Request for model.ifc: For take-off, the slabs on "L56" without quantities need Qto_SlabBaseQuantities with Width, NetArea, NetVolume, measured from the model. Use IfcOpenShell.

First a look at what the model holds.

```python
import ifcopenshell
import ifcopenshell.util.element
import ifcopenshell.util.unit

model = ifcopenshell.open("model.ifc")
print(model.schema)
for unit_type in ("LENGTHUNIT", "AREAUNIT", "VOLUMEUNIT"):
    print(unit_type, ifcopenshell.util.unit.calculate_unit_scale(model, unit_type))
storey = next(s for s in model.by_type("IfcBuildingStorey") if s.Name == "L56")
slabs = [e for e in ifcopenshell.util.element.get_decomposition(storey) if e.is_a("IfcSlab")]
for e in sorted(slabs, key=lambda e: e.id()):
    print(e.id(), e.is_a(), e.Name, list(ifcopenshell.util.element.get_psets(e, qtos_only=True)), sep=" | ")
```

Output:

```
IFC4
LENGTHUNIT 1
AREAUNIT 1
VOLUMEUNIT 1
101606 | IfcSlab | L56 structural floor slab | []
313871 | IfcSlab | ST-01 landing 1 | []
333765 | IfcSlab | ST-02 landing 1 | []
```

```python
import ifcopenshell
import ifcopenshell.api.pset
import ifcopenshell.geom
import ifcopenshell.util.element
import ifcopenshell.util.shape
import ifcopenshell.util.unit

model = ifcopenshell.open("model.ifc")
unit_scale = ifcopenshell.util.unit.calculate_unit_scale(model)
area_scale = ifcopenshell.util.unit.calculate_unit_scale(model, "AREAUNIT")
volume_scale = ifcopenshell.util.unit.calculate_unit_scale(model, "VOLUMEUNIT")
settings = ifcopenshell.geom.settings()

storey = next(s for s in model.by_type("IfcBuildingStorey") if s.Name == "L56")
slabs = [e for e in ifcopenshell.util.element.get_decomposition(storey) if e.is_a("IfcSlab")]

for e in sorted(slabs, key=lambda e: e.id()):
    if ifcopenshell.util.element.get_psets(e, qtos_only=True, should_inherit=False):
        continue
    # Geometry comes back in metres, in the element's own axes.
    shape = ifcopenshell.geom.create_shape(settings, e)
    values = {
        "Width": ifcopenshell.util.shape.get_z(shape.geometry) / unit_scale,
        "NetArea": ifcopenshell.util.shape.get_footprint_area(shape.geometry) / area_scale,
        "NetVolume": ifcopenshell.util.shape.get_volume(shape.geometry) / volume_scale,
    }
    qto = ifcopenshell.api.pset.add_qto(model, product=e, name="Qto_SlabBaseQuantities")
    ifcopenshell.api.pset.edit_qto(model, qto=qto, properties=values)
    print(e.id(), {k: round(v, 3) for k, v in values.items()})

model.write("model-out.ifc")
```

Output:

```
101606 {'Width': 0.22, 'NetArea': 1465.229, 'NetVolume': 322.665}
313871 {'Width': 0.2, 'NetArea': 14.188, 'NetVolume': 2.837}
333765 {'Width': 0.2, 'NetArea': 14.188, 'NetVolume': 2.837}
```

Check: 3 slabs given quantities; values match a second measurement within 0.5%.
